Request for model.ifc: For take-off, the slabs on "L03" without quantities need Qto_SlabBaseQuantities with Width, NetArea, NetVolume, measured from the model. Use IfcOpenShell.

First a look at what the model holds.

```python
import ifcopenshell
import ifcopenshell.util.element
import ifcopenshell.util.unit

model = ifcopenshell.open("model.ifc")
print(model.schema)
for unit_type in ("LENGTHUNIT", "AREAUNIT", "VOLUMEUNIT"):
    print(unit_type, ifcopenshell.util.unit.calculate_unit_scale(model, unit_type))
storey = next(s for s in model.by_type("IfcBuildingStorey") if s.Name == "L03")
slabs = [e for e in ifcopenshell.util.element.get_decomposition(storey) if e.is_a("IfcSlab")]
for e in sorted(slabs, key=lambda e: e.id()):
    print(e.id(), e.is_a(), e.Name, list(ifcopenshell.util.element.get_psets(e, qtos_only=True)), sep=" | ")
```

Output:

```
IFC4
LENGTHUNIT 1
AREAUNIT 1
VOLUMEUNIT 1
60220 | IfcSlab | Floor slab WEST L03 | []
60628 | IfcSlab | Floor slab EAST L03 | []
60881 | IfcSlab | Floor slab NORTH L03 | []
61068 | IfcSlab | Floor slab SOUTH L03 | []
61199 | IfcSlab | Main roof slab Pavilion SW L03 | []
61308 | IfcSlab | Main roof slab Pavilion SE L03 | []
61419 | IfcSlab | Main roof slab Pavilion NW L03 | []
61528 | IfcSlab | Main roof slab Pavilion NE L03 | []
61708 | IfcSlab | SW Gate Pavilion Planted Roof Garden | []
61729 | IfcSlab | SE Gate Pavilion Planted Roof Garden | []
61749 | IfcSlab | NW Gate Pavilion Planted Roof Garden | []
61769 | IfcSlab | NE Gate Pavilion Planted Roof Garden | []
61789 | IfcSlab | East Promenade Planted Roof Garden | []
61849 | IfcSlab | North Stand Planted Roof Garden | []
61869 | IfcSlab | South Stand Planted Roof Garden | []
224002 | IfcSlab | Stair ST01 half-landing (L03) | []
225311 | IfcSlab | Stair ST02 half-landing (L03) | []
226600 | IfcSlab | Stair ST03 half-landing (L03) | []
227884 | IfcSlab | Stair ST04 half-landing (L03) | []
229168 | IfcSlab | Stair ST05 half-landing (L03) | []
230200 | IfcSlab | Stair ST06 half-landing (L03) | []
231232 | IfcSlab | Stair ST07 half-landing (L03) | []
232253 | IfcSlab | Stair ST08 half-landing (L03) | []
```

```python
import ifcopenshell
import ifcopenshell.api.pset
import ifcopenshell.geom
import ifcopenshell.util.element
import ifcopenshell.util.shape
import ifcopenshell.util.unit

model = ifcopenshell.open("model.ifc")
unit_scale = ifcopenshell.util.unit.calculate_unit_scale(model)
area_scale = ifcopenshell.util.unit.calculate_unit_scale(model, "AREAUNIT")
volume_scale = ifcopenshell.util.unit.calculate_unit_scale(model, "VOLUMEUNIT")
settings = ifcopenshell.geom.settings()

storey = next(s for s in model.by_type("IfcBuildingStorey") if s.Name == "L03")
slabs = [e for e in ifcopenshell.util.element.get_decomposition(storey) if e.is_a("IfcSlab")]

for e in sorted(slabs, key=lambda e: e.id()):
    if ifcopenshell.util.element.get_psets(e, qtos_only=True, should_inherit=False):
        continue
    # Geometry comes back in metres, in the element's own axes.
    shape = ifcopenshell.geom.create_shape(settings, e)
    values = {
        "Width": ifcopenshell.util.shape.get_z(shape.geometry) / unit_scale,
        "NetArea": ifcopenshell.util.shape.get_footprint_area(shape.geometry) / area_scale,
        "NetVolume": ifcopenshell.util.shape.get_volume(shape.geometry) / volume_scale,
    }
    qto = ifcopenshell.api.pset.add_qto(model, product=e, name="Qto_SlabBaseQuantities")
    ifcopenshell.api.pset.edit_qto(model, qto=qto, properties=values)
    print(e.id(), {k: round(v, 3) for k, v in values.items()})

model.write("model-out.ifc")
```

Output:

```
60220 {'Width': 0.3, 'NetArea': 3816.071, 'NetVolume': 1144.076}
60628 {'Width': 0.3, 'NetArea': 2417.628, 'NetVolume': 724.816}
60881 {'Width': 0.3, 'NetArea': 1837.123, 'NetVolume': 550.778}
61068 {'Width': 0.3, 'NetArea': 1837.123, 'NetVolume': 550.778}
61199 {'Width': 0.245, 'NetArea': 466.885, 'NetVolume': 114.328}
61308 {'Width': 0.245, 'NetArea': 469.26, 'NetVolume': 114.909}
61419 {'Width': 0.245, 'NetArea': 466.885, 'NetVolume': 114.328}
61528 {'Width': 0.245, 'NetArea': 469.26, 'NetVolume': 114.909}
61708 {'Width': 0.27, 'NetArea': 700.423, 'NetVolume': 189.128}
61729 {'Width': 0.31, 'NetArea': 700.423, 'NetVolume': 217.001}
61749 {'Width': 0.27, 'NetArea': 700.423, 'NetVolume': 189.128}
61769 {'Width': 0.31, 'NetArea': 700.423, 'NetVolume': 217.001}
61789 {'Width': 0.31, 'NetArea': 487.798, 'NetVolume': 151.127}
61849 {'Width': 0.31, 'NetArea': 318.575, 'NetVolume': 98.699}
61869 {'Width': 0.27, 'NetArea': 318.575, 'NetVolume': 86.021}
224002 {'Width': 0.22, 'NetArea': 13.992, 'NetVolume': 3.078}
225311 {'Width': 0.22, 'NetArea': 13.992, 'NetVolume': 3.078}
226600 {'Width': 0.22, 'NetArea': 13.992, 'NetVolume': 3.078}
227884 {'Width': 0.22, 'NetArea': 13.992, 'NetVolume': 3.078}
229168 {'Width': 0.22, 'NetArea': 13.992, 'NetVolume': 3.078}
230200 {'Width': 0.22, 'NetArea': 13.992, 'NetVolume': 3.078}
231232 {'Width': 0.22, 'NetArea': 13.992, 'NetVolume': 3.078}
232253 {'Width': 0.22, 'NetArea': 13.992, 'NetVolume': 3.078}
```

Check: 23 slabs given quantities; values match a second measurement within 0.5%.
